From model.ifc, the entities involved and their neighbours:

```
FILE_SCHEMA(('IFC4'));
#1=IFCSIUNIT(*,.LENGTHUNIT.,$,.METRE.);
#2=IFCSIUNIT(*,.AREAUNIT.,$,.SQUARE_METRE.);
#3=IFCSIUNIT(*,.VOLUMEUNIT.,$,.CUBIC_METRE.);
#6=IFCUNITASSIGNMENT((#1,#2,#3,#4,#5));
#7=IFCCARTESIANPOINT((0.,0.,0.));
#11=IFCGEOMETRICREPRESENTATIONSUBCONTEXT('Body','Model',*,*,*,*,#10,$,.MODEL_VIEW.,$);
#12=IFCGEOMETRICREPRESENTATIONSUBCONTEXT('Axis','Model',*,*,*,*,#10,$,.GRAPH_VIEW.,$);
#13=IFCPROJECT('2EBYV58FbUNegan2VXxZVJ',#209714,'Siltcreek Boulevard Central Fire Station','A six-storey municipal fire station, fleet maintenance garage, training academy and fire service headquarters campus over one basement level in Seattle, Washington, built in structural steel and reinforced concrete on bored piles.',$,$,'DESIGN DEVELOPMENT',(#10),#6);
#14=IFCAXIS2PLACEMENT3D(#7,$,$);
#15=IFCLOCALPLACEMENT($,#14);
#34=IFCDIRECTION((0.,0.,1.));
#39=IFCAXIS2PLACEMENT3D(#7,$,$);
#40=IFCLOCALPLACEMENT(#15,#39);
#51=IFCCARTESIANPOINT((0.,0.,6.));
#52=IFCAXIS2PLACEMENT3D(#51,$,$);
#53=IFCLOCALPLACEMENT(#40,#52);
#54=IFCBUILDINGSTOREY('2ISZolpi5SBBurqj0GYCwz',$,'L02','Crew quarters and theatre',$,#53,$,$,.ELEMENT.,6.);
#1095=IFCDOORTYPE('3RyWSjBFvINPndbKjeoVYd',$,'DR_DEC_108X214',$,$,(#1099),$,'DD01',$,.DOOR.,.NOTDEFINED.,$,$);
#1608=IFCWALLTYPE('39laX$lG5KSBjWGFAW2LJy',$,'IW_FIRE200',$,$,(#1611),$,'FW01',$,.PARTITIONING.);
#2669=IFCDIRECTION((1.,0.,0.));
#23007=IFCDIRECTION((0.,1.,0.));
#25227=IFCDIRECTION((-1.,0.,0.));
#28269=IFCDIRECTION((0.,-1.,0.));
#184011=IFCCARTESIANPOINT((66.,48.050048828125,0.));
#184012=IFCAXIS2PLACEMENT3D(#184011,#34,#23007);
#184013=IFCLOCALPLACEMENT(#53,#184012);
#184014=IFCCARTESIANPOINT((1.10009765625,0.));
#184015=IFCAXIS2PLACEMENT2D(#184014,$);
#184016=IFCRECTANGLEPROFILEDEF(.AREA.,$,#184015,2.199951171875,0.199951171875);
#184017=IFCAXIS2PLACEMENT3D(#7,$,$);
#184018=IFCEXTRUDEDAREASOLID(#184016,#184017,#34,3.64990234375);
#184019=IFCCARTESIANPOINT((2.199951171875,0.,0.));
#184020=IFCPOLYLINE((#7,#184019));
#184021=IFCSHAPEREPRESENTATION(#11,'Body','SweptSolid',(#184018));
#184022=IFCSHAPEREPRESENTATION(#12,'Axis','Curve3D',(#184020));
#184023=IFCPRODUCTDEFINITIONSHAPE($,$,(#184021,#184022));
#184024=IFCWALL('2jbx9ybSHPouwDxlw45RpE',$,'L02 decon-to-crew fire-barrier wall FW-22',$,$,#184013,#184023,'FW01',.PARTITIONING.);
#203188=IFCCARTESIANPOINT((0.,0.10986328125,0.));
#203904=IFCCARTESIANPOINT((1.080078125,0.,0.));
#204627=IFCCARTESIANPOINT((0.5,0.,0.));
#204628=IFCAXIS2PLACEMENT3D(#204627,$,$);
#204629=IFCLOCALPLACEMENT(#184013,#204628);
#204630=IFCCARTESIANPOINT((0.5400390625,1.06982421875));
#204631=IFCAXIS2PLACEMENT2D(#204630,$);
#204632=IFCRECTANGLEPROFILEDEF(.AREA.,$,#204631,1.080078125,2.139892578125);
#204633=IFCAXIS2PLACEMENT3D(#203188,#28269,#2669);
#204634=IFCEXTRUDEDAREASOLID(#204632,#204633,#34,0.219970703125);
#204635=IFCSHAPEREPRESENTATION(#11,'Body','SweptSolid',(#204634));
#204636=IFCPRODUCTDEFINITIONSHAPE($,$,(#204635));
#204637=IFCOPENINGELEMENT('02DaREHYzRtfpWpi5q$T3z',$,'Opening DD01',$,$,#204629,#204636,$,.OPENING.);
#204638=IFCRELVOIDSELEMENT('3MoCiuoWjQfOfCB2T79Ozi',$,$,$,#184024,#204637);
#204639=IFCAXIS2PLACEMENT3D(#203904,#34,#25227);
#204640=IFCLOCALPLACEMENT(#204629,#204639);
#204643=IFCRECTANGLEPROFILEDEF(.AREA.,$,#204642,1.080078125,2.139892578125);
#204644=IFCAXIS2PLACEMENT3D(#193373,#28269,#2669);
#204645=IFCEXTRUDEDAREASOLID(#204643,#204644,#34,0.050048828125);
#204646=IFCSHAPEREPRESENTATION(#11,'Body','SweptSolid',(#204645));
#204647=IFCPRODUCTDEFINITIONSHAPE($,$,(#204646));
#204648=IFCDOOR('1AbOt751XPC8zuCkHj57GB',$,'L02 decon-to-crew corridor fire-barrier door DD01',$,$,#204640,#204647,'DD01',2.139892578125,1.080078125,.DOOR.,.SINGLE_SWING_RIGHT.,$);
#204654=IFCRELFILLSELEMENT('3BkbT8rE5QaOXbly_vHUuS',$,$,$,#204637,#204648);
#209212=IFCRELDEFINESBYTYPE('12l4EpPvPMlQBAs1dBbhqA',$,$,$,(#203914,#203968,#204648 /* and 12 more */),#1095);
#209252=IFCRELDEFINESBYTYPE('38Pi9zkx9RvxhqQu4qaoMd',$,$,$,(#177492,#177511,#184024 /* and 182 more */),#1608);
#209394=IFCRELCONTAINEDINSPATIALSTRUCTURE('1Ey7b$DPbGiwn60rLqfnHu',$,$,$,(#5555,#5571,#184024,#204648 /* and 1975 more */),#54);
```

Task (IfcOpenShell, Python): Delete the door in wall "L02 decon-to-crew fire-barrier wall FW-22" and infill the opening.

```python
import ifcopenshell
import ifcopenshell.api.feature
import ifcopenshell.api.root
import ifcopenshell.geom
import ifcopenshell.util.shape

model = ifcopenshell.open("model.ifc")
settings = ifcopenshell.geom.settings()


def volume(element):
    """Net volume in cubic metres, openings subtracted."""
    shape = ifcopenshell.geom.create_shape(settings, element)
    return ifcopenshell.util.shape.get_volume(shape.geometry)


door = model.by_guid("1AbOt751XPC8zuCkHj57GB")
opening = door.FillsVoids[0].RelatingOpeningElement
wall = opening.VoidsElements[0].RelatingBuildingElement
before = volume(wall)

ifcopenshell.api.root.remove_product(model, product=door)
ifcopenshell.api.feature.remove_feature(model, feature=opening)

after = volume(wall)

print(f"wall volume {before:.3f} -> {after:.3f} m3")

model.write("model_v2.ifc")
```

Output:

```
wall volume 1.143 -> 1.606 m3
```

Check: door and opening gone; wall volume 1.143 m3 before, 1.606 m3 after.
